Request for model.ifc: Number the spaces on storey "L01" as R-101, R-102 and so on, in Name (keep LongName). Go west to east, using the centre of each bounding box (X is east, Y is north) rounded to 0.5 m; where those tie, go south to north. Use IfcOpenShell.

First a look at what the model holds.

```python
import ifcopenshell
import ifcopenshell.util.element
import ifcopenshell.util.placement

model = ifcopenshell.open("model.ifc")
print(model.schema)
storey = next(s for s in model.by_type("IfcBuildingStorey") if s.Name == "L01")
spaces = [e for e in ifcopenshell.util.element.get_decomposition(storey) if e.is_a("IfcSpace")]
for e in sorted(spaces, key=lambda e: e.id()):
    origin = ifcopenshell.util.placement.get_local_placement(e.ObjectPlacement)[:3, 3]
    print(e.id(), e.Name, e.LongName, origin.round(2) + 0.0, sep=" | ")
```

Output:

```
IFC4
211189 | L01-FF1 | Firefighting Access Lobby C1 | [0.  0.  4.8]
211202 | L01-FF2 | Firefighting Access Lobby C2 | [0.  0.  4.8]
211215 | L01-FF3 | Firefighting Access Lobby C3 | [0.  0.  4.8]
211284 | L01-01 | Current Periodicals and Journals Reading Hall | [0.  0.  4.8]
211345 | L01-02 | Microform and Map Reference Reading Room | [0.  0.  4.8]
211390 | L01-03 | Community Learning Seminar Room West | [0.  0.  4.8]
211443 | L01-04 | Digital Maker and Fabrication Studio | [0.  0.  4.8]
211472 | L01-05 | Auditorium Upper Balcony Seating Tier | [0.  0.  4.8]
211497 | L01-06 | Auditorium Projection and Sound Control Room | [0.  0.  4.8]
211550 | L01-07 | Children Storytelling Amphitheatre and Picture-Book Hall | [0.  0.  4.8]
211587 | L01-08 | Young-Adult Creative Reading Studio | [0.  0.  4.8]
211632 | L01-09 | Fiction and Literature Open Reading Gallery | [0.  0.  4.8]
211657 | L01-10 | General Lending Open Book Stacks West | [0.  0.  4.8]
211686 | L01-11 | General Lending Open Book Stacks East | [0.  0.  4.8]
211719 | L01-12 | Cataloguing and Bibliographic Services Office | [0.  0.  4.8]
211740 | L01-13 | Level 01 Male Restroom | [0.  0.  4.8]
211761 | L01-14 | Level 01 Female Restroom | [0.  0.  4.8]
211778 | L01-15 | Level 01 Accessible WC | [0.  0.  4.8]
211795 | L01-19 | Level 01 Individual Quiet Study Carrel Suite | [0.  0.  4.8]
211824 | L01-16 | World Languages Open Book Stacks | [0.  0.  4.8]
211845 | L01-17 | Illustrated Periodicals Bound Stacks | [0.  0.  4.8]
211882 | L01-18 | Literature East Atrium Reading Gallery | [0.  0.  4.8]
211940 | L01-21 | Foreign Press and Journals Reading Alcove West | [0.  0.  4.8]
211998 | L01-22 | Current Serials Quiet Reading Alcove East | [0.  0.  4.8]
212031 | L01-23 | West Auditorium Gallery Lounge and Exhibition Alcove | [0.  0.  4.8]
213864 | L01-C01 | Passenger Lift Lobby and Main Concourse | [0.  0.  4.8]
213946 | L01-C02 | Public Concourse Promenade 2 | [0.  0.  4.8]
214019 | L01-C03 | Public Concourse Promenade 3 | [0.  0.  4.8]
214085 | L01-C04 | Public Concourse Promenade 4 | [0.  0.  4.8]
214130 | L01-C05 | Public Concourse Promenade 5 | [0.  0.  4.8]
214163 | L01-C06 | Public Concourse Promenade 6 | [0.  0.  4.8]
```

```python
import ifcopenshell
import ifcopenshell.geom
import ifcopenshell.util.element
import ifcopenshell.util.shape

model = ifcopenshell.open("model.ifc")
settings = ifcopenshell.geom.settings()
settings.set("use-world-coords", True)


def centre(element):
    shape = ifcopenshell.geom.create_shape(settings, element)
    return ifcopenshell.util.shape.get_bbox_centroid(shape.geometry)


storey = next(s for s in model.by_type("IfcBuildingStorey") if s.Name == "L01")
spaces = [e for e in ifcopenshell.util.element.get_decomposition(storey) if e.is_a("IfcSpace")]

# Insertion points can sit at a corner or the storey origin, so sort by the geometry (in metres).
centres = {e: centre(e) for e in spaces}
spaces.sort(key=lambda e: (round(centres[e][0] / 0.5), centres[e][1]))

for i, e in enumerate(spaces, start=1):
    number = f"R-1{i:02d}"
    e.Name = number
    print(e.id(), number)

model.write("model_edited.ifc")
```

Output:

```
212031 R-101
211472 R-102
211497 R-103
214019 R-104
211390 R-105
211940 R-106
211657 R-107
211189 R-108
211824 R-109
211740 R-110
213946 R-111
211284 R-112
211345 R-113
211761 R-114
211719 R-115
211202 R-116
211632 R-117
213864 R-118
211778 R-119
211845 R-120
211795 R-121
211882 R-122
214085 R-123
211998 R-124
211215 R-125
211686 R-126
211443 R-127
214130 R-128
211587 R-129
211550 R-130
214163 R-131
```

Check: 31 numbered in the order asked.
